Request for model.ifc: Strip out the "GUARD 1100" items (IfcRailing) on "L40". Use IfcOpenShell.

First a look at what the model holds.

```python
import ifcopenshell
import ifcopenshell.util.element

model = ifcopenshell.open("model.ifc")
print(model.schema)
storey = next(s for s in model.by_type("IfcBuildingStorey") if s.Name == "L40")
railings = [e for e in ifcopenshell.util.element.get_decomposition(storey) if e.is_a("IfcRailing")]
seen = {}
for e in railings:
    element_type = ifcopenshell.util.element.get_type(e)
    name = element_type.Name if element_type not in (None, e) else None
    seen[name] = seen.get(name, 0) + 1
for name, count in sorted(seen.items(), key=str):
    print(count, "x", name)
```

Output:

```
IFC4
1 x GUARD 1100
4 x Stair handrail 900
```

```python
import ifcopenshell
import ifcopenshell.api.root
import ifcopenshell.util.element

model = ifcopenshell.open("model.ifc")

storey = next(s for s in model.by_type("IfcBuildingStorey") if s.Name == "L40")
railings = [e for e in ifcopenshell.util.element.get_decomposition(storey) if e.is_a("IfcRailing")]
targets = [e for e in railings if (t := ifcopenshell.util.element.get_type(e)) not in (None, e) and t.Name == "GUARD 1100"]

for e in targets:
    ifcopenshell.api.root.remove_product(model, product=e)
print(len(targets), "removed")

model.write("model_rev.ifc")
```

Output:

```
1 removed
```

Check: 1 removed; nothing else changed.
